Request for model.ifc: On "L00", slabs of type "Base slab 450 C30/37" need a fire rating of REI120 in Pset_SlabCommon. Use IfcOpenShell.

First a look at what the model holds.

```python
import ifcopenshell
import ifcopenshell.util.element

model = ifcopenshell.open("model.ifc")
print(model.schema)
storey = next(s for s in model.by_type("IfcBuildingStorey") if s.Name == "L00")
slabs = [e for e in ifcopenshell.util.element.get_decomposition(storey) if e.is_a("IfcSlab")]
seen = {}
for e in slabs:
    element_type = ifcopenshell.util.element.get_type(e)
    key = (element_type.Name if element_type != e and element_type else None, ifcopenshell.util.element.get_pset(e, "Pset_SlabCommon", "FireRating"))
    seen[key] = seen.get(key, 0) + 1
for (name, value), count in sorted(seen.items(), key=str):
    print(count, "x", name, "|", value)
```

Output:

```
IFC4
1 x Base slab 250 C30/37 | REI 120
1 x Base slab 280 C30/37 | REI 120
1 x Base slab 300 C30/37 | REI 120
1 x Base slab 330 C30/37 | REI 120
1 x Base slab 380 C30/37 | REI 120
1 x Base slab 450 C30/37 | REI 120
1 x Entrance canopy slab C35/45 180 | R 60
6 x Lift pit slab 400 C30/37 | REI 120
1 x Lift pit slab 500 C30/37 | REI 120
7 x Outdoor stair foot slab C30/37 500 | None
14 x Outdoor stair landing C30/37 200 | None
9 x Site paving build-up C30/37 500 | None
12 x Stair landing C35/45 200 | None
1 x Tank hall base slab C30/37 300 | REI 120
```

```python
import ifcopenshell
import ifcopenshell.api.pset
import ifcopenshell.util.element

model = ifcopenshell.open("model.ifc")

storey = next(s for s in model.by_type("IfcBuildingStorey") if s.Name == "L00")
slabs = [e for e in ifcopenshell.util.element.get_decomposition(storey) if e.is_a("IfcSlab")]

count = 0
for e in slabs:
    element_type = ifcopenshell.util.element.get_type(e)
    if element_type in (None, e) or element_type.Name != "Base slab 450 C30/37":
        continue
    # add_pset returns the element's existing set when there is one.
    pset = ifcopenshell.api.pset.add_pset(model, product=e, name="Pset_SlabCommon")
    ifcopenshell.api.pset.edit_pset(model, pset=pset, properties={"FireRating": "REI120"})
    count += 1

print(count, "slabs updated")

model.write("model_edited.ifc")
```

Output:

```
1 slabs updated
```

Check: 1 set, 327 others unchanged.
